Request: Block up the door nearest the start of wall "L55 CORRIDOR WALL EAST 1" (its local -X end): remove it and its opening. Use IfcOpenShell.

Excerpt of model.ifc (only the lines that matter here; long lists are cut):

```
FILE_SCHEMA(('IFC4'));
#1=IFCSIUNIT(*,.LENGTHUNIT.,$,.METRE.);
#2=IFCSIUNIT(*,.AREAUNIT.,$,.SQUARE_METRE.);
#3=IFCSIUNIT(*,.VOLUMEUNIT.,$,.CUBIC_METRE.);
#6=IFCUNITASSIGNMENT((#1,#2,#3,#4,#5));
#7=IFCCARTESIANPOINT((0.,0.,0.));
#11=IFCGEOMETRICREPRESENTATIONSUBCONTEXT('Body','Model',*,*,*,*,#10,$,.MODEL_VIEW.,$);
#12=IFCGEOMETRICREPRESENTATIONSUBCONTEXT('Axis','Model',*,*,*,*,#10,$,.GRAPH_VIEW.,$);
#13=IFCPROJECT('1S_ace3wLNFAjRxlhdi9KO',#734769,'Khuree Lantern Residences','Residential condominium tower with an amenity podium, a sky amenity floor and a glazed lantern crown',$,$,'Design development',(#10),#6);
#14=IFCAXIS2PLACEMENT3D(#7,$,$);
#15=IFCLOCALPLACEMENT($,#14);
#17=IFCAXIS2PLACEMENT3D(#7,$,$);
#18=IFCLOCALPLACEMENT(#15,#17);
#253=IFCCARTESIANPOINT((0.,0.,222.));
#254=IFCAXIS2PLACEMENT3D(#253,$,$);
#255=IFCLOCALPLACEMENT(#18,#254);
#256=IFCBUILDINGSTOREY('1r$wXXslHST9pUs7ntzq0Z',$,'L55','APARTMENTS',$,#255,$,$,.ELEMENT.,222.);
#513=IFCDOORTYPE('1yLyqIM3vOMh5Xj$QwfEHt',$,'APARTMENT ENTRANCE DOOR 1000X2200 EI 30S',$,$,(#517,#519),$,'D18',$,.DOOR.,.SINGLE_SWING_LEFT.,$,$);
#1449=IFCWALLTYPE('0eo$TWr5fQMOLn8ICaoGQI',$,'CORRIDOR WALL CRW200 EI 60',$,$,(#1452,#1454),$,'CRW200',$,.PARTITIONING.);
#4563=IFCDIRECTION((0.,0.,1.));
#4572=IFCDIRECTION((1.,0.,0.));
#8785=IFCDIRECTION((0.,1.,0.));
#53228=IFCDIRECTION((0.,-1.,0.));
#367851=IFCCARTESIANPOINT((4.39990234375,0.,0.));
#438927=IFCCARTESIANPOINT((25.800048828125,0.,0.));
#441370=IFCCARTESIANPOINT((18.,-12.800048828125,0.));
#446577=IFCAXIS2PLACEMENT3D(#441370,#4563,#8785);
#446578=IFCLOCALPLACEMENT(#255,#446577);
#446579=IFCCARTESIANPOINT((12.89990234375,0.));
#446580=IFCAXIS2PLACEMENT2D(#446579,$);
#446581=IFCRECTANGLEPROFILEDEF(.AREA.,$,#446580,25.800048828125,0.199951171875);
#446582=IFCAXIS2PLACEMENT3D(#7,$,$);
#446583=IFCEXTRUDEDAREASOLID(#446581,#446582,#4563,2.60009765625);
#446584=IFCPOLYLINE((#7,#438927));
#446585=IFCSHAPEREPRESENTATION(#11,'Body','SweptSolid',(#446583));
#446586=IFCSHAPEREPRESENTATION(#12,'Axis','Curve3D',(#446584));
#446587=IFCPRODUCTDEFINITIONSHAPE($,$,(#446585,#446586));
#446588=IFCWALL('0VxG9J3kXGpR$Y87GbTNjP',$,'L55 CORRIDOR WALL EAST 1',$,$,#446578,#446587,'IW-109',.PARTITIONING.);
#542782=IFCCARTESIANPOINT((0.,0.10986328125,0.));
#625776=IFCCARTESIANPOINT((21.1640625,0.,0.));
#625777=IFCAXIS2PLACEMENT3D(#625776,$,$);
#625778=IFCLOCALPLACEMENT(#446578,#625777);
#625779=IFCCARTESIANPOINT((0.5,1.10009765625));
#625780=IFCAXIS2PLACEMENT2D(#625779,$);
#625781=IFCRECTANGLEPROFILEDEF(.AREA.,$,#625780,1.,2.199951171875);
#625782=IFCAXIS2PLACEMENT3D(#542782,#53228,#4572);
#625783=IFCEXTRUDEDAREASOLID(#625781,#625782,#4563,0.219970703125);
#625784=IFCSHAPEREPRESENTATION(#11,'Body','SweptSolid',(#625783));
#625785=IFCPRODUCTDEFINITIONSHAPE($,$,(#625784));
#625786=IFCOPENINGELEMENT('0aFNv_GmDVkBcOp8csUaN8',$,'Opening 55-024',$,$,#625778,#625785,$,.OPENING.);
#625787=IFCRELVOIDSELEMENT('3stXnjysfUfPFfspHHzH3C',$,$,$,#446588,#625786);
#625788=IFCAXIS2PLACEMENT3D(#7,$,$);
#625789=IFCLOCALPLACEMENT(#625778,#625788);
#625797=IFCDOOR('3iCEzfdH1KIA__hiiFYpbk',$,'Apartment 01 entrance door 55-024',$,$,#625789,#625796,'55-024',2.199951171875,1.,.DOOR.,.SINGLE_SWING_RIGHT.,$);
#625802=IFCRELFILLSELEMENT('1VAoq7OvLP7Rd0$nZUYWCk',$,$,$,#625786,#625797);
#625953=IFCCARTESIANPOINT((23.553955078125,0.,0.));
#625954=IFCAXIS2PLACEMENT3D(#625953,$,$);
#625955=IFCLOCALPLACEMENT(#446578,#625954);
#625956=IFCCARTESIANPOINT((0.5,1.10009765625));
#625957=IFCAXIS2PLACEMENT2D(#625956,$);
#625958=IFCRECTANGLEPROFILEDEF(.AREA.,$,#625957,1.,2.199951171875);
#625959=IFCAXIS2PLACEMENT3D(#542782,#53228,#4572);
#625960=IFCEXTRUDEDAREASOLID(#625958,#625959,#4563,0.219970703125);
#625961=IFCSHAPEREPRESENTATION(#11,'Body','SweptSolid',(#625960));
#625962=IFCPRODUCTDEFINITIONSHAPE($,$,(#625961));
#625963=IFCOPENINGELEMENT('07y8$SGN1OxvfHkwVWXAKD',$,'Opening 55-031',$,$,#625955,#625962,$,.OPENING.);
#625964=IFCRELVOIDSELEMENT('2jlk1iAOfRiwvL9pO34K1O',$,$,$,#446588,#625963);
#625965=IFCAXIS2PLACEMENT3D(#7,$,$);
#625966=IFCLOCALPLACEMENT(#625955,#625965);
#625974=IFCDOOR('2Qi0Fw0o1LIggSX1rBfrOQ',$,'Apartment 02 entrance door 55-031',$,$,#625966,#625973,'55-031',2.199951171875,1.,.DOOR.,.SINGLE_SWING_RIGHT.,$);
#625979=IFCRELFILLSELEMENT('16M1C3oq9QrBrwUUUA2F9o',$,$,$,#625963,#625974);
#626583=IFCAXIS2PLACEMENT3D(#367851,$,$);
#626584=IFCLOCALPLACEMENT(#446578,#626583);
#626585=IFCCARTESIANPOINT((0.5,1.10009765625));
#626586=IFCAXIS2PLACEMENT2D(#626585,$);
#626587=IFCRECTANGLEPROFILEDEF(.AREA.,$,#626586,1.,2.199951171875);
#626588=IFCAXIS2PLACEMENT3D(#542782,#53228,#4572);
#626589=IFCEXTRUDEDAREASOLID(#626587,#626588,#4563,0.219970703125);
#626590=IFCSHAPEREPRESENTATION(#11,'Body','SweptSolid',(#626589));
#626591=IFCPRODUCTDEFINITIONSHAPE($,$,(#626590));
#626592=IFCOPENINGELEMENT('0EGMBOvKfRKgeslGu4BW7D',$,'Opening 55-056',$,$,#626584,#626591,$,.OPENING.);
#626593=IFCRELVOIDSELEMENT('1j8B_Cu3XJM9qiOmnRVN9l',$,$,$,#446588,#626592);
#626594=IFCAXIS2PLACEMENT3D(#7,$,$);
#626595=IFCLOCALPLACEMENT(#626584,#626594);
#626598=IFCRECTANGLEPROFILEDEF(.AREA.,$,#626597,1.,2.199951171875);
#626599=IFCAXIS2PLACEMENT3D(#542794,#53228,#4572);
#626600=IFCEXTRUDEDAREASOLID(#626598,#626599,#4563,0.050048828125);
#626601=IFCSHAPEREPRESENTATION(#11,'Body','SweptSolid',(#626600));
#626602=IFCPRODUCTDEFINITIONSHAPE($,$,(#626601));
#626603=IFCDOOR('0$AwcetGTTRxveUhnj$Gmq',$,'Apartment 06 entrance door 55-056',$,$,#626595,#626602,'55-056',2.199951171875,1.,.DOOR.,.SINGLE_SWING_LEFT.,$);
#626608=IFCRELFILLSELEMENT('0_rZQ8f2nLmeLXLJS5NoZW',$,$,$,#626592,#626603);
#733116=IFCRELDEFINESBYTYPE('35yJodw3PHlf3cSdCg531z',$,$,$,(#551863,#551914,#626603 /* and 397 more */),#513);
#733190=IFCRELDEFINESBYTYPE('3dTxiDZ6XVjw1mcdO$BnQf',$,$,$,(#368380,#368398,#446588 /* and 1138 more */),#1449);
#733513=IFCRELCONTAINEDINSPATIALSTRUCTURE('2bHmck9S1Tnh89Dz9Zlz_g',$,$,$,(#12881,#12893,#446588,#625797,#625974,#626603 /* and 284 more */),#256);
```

```python
import ifcopenshell
import ifcopenshell.api.feature
import ifcopenshell.api.root
import ifcopenshell.geom
import ifcopenshell.util.shape

model = ifcopenshell.open("model.ifc")
settings = ifcopenshell.geom.settings()


def volume(element):
    """Net volume in cubic metres, openings subtracted."""
    shape = ifcopenshell.geom.create_shape(settings, element)
    return ifcopenshell.util.shape.get_volume(shape.geometry)


door = model.by_guid("0$AwcetGTTRxveUhnj$Gmq")
opening = door.FillsVoids[0].RelatingOpeningElement
wall = opening.VoidsElements[0].RelatingBuildingElement
before = volume(wall)

ifcopenshell.api.root.remove_product(model, product=door)
ifcopenshell.api.feature.remove_feature(model, feature=opening)

after = volume(wall)

print(f"wall volume {before:.3f} -> {after:.3f} m3")

model.write("model_v2.ifc")
```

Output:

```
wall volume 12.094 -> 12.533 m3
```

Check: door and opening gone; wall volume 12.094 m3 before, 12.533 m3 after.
